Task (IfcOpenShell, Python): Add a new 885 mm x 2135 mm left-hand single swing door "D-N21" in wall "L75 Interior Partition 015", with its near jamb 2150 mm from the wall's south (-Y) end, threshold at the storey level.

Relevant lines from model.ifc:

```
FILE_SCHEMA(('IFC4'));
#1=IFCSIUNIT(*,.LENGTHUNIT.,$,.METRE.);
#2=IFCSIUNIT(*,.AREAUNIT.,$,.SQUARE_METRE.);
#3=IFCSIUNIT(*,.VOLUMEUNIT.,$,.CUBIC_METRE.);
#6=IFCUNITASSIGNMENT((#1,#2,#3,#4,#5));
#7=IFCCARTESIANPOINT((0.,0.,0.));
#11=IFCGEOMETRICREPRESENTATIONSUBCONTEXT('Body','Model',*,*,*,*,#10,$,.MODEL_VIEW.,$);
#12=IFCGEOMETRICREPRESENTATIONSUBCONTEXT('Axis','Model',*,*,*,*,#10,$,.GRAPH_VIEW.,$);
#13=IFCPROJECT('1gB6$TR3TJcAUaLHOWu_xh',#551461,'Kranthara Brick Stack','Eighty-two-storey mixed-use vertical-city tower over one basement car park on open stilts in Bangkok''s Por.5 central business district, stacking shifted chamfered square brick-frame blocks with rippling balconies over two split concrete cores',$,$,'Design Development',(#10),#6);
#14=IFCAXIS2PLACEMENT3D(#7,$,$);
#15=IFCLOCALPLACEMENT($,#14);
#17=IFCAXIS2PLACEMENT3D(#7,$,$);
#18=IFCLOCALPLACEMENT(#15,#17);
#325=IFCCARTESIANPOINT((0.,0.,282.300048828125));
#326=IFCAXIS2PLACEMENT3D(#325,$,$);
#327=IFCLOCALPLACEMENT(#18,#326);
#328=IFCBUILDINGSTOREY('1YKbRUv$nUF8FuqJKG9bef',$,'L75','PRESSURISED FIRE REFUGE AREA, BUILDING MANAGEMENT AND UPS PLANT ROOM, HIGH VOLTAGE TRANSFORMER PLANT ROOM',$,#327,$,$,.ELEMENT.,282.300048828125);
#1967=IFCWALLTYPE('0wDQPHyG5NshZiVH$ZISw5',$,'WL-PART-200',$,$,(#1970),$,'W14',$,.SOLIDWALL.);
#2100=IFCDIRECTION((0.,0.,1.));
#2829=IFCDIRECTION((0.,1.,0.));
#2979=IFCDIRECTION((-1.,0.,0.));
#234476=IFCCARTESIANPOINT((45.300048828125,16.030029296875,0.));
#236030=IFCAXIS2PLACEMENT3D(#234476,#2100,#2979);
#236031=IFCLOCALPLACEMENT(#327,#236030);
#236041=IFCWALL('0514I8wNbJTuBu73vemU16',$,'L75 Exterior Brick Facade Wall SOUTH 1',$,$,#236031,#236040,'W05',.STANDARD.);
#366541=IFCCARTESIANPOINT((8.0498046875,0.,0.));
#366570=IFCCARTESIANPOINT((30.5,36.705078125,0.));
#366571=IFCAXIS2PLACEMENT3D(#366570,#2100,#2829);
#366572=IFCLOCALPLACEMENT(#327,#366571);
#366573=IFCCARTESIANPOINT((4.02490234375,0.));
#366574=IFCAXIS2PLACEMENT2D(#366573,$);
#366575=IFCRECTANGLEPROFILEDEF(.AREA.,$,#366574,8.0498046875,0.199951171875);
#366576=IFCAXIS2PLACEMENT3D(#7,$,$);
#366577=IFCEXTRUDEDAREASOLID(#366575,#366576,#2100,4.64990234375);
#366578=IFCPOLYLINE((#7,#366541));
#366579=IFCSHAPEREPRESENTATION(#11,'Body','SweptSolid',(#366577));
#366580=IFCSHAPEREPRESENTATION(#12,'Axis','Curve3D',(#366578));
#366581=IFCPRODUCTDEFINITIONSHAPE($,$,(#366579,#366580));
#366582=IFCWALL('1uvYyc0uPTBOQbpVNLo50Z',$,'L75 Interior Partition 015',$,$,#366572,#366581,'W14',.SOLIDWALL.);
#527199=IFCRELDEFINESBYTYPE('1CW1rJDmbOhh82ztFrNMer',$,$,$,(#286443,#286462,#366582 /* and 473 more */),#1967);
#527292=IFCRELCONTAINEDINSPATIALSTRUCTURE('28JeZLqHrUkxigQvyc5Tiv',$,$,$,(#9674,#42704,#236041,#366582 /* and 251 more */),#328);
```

```python
import numpy as np
import ifcopenshell
import ifcopenshell.api.feature
import ifcopenshell.api.geometry
import ifcopenshell.api.root
import ifcopenshell.api.spatial
import ifcopenshell.geom
import ifcopenshell.util.element
import ifcopenshell.util.placement
import ifcopenshell.util.representation
import ifcopenshell.util.shape
import ifcopenshell.util.unit

model = ifcopenshell.open("model.ifc")
unit_scale = ifcopenshell.util.unit.calculate_unit_scale(model)
settings = ifcopenshell.geom.settings()


def volume(element):
    """Net volume in cubic metres, openings subtracted."""
    shape = ifcopenshell.geom.create_shape(settings, element)
    return ifcopenshell.util.shape.get_volume(shape.geometry)


wall = model.by_guid("1uvYyc0uPTBOQbpVNLo50Z")
storey = ifcopenshell.util.element.get_container(wall, ifc_class="IfcBuildingStorey")
context = ifcopenshell.util.representation.get_context(model, "Model", "Body", "MODEL_VIEW")
before = volume(wall)

width, height, from_end, sill = 0.885, 2.135, 2.15, 0.0  # metres

# The wall runs along its own X axis, and the end named is its -X end.
wall_shape = ifcopenshell.geom.create_shape(settings, wall)
x, y, z = ifcopenshell.util.shape.get_vertices(wall_shape.geometry).T
start = x.min() + from_end
face, thickness = float(y.min()), float(y.max() - y.min())
wall_matrix = ifcopenshell.util.placement.get_local_placement(wall.ObjectPlacement)
level = ifcopenshell.util.placement.get_local_placement(storey.ObjectPlacement)[2, 3]


def in_wall(x, y):
    """Placement at x, y metres in the wall's axes, at sill height."""
    matrix = wall_matrix.copy()
    matrix[:, 3] = wall_matrix @ np.array([x / unit_scale, y / unit_scale, 0.0, 1.0])
    matrix[2, 3] = level + sill / unit_scale
    return matrix


# Opening: a box that overshoots both wall faces by 50 mm.
opening = ifcopenshell.api.root.create_entity(model, ifc_class="IfcOpeningElement", predefined_type="OPENING")
box = ifcopenshell.api.geometry.add_wall_representation(
    model, context=context, length=width, height=height, thickness=thickness + 0.1
)
ifcopenshell.api.geometry.assign_representation(model, product=opening, representation=box)
ifcopenshell.api.geometry.edit_object_placement(model, product=opening, matrix=in_wall(start, face - 0.05), is_si=False)
ifcopenshell.api.feature.add_feature(model, feature=opening, element=wall)

door = ifcopenshell.api.root.create_entity(model, ifc_class="IfcDoor", name="D-N21", predefined_type="DOOR")
door.OverallWidth, door.OverallHeight = width / unit_scale, height / unit_scale
door.OperationType = "SINGLE_SWING_LEFT"
body = ifcopenshell.api.geometry.add_door_representation(
    model,
    context=context,
    overall_width=door.OverallWidth,
    overall_height=door.OverallHeight,
    operation_type="SINGLE_SWING_LEFT",
    lining_properties={"LiningDepth": thickness / unit_scale, "ThresholdDepth": thickness / unit_scale},
)
ifcopenshell.api.geometry.assign_representation(model, product=door, representation=body)
ifcopenshell.api.spatial.assign_container(model, products=[door], relating_structure=storey)
ifcopenshell.api.feature.add_filling(model, opening=opening, element=door)

# The lining spans the wall, so the door starts at the wall face.
ifcopenshell.api.geometry.edit_object_placement(model, product=door, matrix=in_wall(start, face), is_si=False)

after = volume(wall)

print(f"wall volume {before:.3f} -> {after:.3f} m3")

model.write("model_edited.ifc")
```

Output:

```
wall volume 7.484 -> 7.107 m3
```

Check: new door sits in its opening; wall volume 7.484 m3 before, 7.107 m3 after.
